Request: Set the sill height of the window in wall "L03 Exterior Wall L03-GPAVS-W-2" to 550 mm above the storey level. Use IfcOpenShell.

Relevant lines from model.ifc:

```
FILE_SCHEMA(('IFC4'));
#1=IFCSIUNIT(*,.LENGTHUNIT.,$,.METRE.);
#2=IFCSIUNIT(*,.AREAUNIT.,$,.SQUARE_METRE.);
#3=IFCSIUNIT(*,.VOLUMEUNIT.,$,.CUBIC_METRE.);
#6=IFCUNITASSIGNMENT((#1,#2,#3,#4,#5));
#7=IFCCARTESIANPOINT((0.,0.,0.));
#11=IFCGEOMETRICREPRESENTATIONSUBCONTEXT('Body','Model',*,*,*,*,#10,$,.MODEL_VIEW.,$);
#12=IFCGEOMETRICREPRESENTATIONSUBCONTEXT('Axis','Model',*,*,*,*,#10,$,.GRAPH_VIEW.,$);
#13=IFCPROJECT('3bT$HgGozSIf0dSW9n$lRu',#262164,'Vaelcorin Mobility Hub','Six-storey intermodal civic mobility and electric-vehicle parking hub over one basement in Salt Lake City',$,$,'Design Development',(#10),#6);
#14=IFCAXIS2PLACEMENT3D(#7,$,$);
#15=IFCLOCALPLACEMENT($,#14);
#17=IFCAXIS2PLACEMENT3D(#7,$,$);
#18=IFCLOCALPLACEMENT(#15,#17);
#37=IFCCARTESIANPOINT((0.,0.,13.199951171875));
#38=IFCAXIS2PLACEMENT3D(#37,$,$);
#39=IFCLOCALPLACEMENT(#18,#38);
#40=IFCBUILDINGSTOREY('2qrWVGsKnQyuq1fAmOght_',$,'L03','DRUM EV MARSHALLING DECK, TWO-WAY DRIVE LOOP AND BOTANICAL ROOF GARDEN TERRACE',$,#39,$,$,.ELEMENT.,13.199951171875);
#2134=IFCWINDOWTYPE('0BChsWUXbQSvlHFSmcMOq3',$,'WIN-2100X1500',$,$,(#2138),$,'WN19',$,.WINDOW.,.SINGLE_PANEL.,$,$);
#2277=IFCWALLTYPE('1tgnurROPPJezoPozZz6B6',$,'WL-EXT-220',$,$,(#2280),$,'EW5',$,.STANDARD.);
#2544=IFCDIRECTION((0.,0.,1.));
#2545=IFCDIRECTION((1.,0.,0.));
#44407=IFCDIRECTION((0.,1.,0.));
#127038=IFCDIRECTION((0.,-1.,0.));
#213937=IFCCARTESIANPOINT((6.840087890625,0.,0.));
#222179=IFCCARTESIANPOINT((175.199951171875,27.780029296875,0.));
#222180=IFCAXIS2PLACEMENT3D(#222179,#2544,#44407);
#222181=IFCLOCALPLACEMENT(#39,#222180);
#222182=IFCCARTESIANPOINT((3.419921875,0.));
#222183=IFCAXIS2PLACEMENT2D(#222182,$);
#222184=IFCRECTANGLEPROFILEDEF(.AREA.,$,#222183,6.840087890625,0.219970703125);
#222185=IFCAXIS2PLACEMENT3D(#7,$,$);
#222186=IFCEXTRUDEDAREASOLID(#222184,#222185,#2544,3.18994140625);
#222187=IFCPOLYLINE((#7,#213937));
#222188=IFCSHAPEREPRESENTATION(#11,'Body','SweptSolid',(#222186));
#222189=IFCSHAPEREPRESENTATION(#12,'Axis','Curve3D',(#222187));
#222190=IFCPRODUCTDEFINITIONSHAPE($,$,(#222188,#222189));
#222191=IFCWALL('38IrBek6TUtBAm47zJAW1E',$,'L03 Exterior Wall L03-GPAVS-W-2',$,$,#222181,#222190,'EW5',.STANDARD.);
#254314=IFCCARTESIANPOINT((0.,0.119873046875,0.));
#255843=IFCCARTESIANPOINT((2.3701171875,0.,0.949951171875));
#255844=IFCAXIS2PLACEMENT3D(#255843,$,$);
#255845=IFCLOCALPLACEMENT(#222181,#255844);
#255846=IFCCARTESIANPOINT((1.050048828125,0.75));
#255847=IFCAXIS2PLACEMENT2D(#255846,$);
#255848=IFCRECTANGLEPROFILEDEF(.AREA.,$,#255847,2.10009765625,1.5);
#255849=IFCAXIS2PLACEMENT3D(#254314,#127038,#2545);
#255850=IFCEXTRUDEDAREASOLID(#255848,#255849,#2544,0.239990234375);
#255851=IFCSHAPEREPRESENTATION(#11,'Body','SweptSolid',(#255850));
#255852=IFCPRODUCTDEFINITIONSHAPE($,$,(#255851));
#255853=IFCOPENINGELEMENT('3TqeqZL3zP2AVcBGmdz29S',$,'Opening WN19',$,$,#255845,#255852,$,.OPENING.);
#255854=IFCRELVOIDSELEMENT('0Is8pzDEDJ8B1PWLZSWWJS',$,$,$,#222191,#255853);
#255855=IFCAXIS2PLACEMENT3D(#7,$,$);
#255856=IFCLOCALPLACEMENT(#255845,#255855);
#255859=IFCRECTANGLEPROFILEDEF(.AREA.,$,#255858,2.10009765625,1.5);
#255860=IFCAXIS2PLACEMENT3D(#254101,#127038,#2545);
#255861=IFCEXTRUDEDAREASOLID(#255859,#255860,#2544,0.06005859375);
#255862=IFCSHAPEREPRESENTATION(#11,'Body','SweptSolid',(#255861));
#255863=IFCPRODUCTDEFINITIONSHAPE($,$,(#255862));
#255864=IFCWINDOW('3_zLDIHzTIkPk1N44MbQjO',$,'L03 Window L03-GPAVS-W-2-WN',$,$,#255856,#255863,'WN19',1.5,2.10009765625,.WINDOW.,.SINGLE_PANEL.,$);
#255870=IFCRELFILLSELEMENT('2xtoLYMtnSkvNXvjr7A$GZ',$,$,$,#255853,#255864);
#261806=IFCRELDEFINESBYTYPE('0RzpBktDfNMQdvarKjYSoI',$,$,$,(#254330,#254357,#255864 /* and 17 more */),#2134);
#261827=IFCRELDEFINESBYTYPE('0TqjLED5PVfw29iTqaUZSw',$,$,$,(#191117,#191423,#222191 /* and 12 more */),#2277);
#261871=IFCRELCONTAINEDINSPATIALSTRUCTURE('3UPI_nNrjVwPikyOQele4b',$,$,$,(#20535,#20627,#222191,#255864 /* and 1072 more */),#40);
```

```python
import numpy as np
import ifcopenshell
import ifcopenshell.api.geometry
import ifcopenshell.geom
import ifcopenshell.util.element
import ifcopenshell.util.placement
import ifcopenshell.util.shape
import ifcopenshell.util.unit

model = ifcopenshell.open("model.ifc")
unit_scale = ifcopenshell.util.unit.calculate_unit_scale(model)

window = model.by_guid("3_zLDIHzTIkPk1N44MbQjO")
opening = window.FillsVoids[0].RelatingOpeningElement
storey = ifcopenshell.util.element.get_container(window, ifc_class="IfcBuildingStorey")
level = ifcopenshell.util.placement.get_local_placement(storey.ObjectPlacement)[2, 3]

# The opening's origin need not be at the sill, so measure its lowest point.
shape = ifcopenshell.geom.create_shape(ifcopenshell.geom.settings(), opening)
bottom = ifcopenshell.util.shape.get_shape_bottom_elevation(shape, shape.geometry) / unit_scale
dz = level + 0.55 - bottom

shift = np.array([0.0, 0.0, dz])
# The window is placed relative to its opening, so it follows when the opening moves.
matrix = ifcopenshell.util.placement.get_local_placement(opening.ObjectPlacement)
matrix[:3, 3] += shift
ifcopenshell.api.geometry.edit_object_placement(
    model, product=opening, matrix=matrix, is_si=False, should_transform_children=True
)

print(f"moved by {dz * unit_scale:+.3f} m")

model.write("model-out.ifc")
```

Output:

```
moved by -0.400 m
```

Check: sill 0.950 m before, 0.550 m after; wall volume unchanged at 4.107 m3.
